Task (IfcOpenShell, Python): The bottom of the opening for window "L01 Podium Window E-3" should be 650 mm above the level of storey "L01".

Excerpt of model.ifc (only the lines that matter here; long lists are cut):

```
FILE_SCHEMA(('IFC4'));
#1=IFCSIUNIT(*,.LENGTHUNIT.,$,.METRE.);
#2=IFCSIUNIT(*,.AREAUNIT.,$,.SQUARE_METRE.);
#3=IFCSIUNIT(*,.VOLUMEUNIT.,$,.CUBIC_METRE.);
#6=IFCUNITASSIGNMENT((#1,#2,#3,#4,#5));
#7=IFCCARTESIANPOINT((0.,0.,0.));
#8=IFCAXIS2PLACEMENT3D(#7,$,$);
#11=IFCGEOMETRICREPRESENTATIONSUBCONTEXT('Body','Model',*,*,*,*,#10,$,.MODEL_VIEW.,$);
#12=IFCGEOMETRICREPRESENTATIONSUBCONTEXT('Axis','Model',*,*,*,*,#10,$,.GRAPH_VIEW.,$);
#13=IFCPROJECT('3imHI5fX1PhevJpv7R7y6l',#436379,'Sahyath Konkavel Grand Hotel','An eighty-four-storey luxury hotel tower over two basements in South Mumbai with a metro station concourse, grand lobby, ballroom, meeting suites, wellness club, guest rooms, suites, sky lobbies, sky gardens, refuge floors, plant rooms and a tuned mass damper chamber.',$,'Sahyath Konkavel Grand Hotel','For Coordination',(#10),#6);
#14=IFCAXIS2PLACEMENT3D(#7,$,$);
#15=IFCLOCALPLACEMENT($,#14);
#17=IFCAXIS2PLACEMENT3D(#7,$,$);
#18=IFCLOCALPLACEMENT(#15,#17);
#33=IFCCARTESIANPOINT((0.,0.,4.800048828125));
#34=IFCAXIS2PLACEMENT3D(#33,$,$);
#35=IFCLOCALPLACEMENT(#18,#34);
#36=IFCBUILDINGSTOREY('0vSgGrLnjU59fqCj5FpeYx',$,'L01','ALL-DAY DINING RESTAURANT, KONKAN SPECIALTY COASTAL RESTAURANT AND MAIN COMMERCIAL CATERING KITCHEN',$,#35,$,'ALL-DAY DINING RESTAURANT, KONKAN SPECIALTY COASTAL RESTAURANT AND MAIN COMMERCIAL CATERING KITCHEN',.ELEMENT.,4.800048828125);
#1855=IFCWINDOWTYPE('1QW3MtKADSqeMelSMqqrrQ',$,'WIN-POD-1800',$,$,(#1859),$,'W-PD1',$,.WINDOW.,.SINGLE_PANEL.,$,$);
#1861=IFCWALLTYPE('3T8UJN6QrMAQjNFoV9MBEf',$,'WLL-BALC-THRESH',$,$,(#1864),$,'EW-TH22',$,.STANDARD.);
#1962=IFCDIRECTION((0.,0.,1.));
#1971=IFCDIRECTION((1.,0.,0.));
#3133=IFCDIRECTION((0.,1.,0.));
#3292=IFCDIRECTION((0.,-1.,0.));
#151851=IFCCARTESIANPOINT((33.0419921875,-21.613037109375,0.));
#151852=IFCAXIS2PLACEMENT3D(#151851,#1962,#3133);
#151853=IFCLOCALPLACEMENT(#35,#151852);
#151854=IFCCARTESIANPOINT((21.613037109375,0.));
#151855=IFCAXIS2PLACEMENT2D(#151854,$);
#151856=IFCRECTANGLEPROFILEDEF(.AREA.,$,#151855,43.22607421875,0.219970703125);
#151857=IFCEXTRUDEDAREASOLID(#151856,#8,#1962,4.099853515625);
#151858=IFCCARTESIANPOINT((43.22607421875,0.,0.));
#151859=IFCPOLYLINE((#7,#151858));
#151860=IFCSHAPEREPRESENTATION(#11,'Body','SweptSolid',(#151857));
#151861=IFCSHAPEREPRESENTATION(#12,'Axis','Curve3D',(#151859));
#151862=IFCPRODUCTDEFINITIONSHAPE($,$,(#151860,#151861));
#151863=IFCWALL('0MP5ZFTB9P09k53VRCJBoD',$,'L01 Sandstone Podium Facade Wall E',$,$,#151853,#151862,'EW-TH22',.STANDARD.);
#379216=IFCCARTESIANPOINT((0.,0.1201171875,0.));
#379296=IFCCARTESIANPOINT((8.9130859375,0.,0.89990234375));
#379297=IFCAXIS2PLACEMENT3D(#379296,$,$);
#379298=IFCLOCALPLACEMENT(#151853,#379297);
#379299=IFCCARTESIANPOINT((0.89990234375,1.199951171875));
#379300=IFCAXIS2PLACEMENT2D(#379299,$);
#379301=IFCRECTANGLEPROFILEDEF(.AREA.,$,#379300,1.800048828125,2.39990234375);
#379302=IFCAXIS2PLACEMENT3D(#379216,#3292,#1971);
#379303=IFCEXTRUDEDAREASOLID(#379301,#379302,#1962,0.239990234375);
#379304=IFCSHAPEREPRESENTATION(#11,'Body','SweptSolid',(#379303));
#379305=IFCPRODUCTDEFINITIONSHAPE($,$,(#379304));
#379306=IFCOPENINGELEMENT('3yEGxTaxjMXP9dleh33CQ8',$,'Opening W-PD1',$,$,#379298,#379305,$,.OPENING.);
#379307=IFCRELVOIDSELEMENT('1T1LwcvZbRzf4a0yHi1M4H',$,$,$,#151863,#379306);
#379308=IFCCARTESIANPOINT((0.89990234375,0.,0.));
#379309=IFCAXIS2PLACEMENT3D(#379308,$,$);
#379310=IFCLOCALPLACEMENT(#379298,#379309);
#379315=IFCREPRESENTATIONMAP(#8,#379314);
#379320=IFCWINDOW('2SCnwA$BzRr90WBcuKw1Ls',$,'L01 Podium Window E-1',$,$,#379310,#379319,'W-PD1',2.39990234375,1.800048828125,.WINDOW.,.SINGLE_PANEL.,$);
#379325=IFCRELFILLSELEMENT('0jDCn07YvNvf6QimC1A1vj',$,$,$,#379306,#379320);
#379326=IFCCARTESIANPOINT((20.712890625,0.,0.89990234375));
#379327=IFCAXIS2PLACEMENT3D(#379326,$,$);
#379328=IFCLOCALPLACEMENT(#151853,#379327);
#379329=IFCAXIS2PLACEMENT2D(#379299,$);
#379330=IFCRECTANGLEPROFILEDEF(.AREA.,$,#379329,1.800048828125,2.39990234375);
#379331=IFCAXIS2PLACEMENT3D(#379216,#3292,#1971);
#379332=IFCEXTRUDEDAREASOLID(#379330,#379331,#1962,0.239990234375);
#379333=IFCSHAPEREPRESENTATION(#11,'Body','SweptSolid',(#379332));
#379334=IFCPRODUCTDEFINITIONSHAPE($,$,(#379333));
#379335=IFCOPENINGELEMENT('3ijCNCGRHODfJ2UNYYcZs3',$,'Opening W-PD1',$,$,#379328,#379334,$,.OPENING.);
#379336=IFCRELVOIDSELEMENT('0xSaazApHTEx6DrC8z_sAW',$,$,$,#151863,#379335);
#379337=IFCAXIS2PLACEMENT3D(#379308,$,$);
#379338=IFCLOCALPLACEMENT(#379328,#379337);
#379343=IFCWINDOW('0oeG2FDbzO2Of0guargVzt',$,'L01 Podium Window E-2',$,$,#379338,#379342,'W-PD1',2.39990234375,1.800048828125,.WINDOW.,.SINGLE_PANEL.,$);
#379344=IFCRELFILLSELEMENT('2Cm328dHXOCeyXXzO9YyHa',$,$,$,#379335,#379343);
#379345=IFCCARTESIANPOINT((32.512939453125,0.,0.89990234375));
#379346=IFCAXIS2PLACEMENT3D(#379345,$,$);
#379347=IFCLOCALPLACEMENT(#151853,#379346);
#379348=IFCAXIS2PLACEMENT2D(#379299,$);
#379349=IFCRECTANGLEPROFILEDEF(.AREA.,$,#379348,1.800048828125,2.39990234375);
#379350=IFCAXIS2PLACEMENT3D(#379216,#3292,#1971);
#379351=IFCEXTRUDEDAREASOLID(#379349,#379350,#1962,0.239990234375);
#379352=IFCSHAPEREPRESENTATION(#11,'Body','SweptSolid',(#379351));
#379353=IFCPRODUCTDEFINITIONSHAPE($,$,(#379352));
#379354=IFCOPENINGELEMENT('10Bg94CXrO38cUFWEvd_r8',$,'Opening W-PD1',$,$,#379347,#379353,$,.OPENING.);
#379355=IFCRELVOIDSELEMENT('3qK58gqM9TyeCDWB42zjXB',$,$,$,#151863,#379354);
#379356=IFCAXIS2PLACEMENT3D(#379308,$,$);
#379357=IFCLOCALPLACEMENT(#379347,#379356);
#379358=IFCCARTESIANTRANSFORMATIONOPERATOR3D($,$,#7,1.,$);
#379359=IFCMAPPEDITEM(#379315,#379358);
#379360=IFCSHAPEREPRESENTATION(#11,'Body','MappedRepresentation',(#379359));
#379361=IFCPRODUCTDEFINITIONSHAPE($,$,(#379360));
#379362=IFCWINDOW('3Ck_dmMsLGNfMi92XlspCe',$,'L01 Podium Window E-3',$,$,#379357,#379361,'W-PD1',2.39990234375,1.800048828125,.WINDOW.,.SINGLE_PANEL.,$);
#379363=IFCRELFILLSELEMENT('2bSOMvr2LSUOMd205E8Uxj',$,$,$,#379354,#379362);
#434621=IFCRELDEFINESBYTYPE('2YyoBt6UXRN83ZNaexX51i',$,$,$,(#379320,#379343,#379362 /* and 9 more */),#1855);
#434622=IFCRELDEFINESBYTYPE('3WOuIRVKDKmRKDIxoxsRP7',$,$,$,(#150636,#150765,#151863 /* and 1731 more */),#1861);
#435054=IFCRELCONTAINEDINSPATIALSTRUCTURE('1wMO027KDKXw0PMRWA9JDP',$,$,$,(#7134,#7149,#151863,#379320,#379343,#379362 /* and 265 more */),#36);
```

```python
import numpy as np
import ifcopenshell
import ifcopenshell.api.geometry
import ifcopenshell.geom
import ifcopenshell.util.element
import ifcopenshell.util.placement
import ifcopenshell.util.shape
import ifcopenshell.util.unit

model = ifcopenshell.open("model.ifc")
unit_scale = ifcopenshell.util.unit.calculate_unit_scale(model)

window = model.by_guid("3Ck_dmMsLGNfMi92XlspCe")
opening = window.FillsVoids[0].RelatingOpeningElement
storey = ifcopenshell.util.element.get_container(window, ifc_class="IfcBuildingStorey")
level = ifcopenshell.util.placement.get_local_placement(storey.ObjectPlacement)[2, 3]

# The opening's origin need not be at the sill, so measure its lowest point.
shape = ifcopenshell.geom.create_shape(ifcopenshell.geom.settings(), opening)
bottom = ifcopenshell.util.shape.get_shape_bottom_elevation(shape, shape.geometry) / unit_scale
dz = level + 0.65 / unit_scale - bottom

shift = np.array([0.0, 0.0, dz])
# The window is placed relative to its opening, so it follows when the opening moves.
matrix = ifcopenshell.util.placement.get_local_placement(opening.ObjectPlacement)
matrix[:3, 3] += shift
ifcopenshell.api.geometry.edit_object_placement(
    model, product=opening, matrix=matrix, is_si=False, should_transform_children=True
)

print(f"moved by {dz * unit_scale:+.3f} m")

model.write("model_v2.ifc")
```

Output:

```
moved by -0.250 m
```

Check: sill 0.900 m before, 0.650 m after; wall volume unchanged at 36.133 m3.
